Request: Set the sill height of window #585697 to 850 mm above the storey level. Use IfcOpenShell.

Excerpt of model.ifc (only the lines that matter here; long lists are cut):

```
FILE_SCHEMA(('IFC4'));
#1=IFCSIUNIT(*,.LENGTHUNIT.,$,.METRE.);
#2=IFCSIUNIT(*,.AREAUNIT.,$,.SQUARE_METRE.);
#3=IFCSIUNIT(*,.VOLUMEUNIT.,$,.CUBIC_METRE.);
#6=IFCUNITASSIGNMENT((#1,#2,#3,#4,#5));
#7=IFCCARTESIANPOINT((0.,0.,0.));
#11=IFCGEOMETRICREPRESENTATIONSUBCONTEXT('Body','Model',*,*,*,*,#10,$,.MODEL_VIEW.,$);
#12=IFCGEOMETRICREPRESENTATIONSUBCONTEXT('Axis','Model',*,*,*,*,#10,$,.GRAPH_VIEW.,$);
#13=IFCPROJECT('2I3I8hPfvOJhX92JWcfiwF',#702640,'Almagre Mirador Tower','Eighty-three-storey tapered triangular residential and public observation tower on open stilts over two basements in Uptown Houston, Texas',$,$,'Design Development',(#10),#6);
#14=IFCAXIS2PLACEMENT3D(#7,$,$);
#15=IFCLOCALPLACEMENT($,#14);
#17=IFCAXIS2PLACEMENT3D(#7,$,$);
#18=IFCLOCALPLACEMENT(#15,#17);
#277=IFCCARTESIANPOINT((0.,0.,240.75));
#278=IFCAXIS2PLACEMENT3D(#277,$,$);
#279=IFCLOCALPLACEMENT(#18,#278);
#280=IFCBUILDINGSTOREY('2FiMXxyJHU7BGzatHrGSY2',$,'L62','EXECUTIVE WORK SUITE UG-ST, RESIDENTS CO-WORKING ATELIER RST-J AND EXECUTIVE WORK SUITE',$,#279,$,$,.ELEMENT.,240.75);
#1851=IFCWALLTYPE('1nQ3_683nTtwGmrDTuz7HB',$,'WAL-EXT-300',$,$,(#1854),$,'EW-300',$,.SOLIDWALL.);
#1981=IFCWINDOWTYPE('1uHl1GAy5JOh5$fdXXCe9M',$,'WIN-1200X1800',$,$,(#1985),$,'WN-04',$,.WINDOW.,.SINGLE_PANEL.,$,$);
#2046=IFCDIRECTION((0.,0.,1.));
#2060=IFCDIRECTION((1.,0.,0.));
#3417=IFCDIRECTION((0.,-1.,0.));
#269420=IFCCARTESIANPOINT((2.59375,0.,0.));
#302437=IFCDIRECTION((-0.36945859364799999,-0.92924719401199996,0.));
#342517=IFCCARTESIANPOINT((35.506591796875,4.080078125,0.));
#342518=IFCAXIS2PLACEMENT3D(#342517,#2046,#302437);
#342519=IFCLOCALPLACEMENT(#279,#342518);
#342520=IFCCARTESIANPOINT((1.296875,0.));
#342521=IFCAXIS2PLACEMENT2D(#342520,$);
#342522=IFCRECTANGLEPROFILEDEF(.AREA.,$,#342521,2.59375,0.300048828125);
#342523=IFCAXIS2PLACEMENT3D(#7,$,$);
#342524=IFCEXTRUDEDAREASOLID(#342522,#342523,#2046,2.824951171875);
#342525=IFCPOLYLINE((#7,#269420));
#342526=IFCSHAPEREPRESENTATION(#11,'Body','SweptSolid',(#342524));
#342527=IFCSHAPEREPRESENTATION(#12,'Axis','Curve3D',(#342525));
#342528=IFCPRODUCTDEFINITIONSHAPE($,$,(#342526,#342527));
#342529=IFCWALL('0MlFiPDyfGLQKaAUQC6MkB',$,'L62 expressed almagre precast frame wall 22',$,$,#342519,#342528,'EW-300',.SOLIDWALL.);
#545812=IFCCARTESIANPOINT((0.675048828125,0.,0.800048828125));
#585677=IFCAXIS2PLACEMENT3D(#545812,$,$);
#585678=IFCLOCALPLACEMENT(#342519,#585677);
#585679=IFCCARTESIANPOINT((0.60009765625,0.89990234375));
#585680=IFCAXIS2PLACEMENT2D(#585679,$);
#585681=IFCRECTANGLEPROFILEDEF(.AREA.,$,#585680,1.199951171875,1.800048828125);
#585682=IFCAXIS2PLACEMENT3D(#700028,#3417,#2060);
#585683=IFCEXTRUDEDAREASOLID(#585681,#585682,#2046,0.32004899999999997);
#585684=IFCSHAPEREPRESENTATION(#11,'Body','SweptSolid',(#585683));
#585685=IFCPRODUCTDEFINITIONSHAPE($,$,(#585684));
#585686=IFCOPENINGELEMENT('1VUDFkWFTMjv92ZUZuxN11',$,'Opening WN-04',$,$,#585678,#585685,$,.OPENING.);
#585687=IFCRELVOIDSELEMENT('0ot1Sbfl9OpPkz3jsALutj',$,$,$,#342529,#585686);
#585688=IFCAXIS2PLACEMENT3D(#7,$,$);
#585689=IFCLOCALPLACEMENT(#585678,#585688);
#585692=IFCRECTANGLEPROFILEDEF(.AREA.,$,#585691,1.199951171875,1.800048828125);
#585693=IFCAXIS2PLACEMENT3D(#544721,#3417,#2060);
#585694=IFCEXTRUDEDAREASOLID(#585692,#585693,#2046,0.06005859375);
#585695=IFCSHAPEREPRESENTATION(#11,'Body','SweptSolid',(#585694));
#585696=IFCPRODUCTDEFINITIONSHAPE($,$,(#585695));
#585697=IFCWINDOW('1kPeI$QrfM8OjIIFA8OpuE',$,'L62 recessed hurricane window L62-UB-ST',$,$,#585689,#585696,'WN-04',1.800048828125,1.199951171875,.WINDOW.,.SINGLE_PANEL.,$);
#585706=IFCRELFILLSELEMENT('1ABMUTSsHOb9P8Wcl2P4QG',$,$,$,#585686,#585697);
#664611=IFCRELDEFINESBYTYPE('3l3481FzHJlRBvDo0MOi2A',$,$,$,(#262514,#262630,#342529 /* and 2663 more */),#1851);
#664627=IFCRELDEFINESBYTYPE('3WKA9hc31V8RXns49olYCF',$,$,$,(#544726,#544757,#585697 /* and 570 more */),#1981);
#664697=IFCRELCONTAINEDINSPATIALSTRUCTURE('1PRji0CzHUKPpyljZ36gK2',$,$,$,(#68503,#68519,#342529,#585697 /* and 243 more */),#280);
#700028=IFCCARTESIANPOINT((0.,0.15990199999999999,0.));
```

```python
import numpy as np
import ifcopenshell
import ifcopenshell.api.geometry
import ifcopenshell.geom
import ifcopenshell.util.element
import ifcopenshell.util.placement
import ifcopenshell.util.shape
import ifcopenshell.util.unit

model = ifcopenshell.open("model.ifc")
unit_scale = ifcopenshell.util.unit.calculate_unit_scale(model)

window = model.by_guid("1kPeI$QrfM8OjIIFA8OpuE")
opening = window.FillsVoids[0].RelatingOpeningElement
storey = ifcopenshell.util.element.get_container(window, ifc_class="IfcBuildingStorey")
level = ifcopenshell.util.placement.get_local_placement(storey.ObjectPlacement)[2, 3]

# The opening's origin need not be at the sill, so measure its lowest point.
shape = ifcopenshell.geom.create_shape(ifcopenshell.geom.settings(), opening)
bottom = ifcopenshell.util.shape.get_shape_bottom_elevation(shape, shape.geometry) / unit_scale
dz = level + 0.85 / unit_scale - bottom

shift = np.array([0.0, 0.0, dz])
# The window is placed relative to its opening, so it follows when the opening moves.
matrix = ifcopenshell.util.placement.get_local_placement(opening.ObjectPlacement)
matrix[:3, 3] += shift
ifcopenshell.api.geometry.edit_object_placement(
    model, product=opening, matrix=matrix, is_si=False, should_transform_children=True
)

print(f"moved by {dz * unit_scale:+.3f} m")

model.write("model_edited.ifc")
```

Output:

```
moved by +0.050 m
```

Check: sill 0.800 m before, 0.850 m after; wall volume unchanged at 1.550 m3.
